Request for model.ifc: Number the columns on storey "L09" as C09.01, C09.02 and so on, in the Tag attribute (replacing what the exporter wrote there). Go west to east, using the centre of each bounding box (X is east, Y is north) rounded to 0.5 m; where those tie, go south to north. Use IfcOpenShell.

First a look at what the model holds.

```python
import ifcopenshell
import ifcopenshell.util.element
import ifcopenshell.util.placement

model = ifcopenshell.open("model.ifc")
print(model.schema)
storey = next(s for s in model.by_type("IfcBuildingStorey") if s.Name == "L09")
columns = [e for e in ifcopenshell.util.element.get_decomposition(storey) if e.is_a("IfcColumn")]
for e in sorted(columns, key=lambda e: e.id()):
    origin = ifcopenshell.util.placement.get_local_placement(e.ObjectPlacement)[:3, 3]
    print(e.id(), e.Tag, e.Name, origin.round(2) + 0.0, sep=" | ")
```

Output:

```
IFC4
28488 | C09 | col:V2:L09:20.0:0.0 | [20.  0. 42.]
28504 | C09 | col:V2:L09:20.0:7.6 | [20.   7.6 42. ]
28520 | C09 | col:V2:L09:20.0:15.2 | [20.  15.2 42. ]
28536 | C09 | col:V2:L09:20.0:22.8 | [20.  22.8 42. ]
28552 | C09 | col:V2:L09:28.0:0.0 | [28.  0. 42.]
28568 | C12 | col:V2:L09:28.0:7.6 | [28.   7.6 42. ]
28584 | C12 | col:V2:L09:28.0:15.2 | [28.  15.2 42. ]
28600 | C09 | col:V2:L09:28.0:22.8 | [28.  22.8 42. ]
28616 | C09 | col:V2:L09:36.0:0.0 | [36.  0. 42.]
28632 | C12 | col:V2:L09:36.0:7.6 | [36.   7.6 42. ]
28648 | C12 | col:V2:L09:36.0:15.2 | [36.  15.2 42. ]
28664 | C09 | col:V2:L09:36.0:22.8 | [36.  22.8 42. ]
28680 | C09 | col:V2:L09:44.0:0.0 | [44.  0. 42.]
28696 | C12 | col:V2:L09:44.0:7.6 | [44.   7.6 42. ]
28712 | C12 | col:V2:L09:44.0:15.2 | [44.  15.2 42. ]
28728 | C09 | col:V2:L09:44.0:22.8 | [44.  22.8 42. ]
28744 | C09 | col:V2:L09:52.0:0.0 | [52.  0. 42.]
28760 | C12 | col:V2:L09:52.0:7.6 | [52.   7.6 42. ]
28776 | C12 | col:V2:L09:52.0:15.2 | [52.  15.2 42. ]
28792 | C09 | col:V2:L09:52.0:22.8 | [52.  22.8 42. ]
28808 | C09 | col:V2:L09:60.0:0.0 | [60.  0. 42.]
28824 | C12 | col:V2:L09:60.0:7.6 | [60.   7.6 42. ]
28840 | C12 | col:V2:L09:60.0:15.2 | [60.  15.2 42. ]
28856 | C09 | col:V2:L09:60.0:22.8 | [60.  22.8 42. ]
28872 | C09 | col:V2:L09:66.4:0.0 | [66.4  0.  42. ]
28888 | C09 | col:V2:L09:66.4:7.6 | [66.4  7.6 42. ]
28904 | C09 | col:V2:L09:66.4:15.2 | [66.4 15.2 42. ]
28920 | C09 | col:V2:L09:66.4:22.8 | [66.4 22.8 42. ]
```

```python
import ifcopenshell
import ifcopenshell.geom
import ifcopenshell.util.element
import ifcopenshell.util.shape

model = ifcopenshell.open("model.ifc")
settings = ifcopenshell.geom.settings()
settings.set("use-world-coords", True)


def centre(element):
    shape = ifcopenshell.geom.create_shape(settings, element)
    return ifcopenshell.util.shape.get_bbox_centroid(shape.geometry)


storey = next(s for s in model.by_type("IfcBuildingStorey") if s.Name == "L09")
columns = [e for e in ifcopenshell.util.element.get_decomposition(storey) if e.is_a("IfcColumn")]

# Insertion points can sit at a corner or the storey origin, so sort by the geometry (in metres).
centres = {e: centre(e) for e in columns}
columns.sort(key=lambda e: (round(centres[e][0] / 0.5), centres[e][1]))

for i, e in enumerate(columns, start=1):
    number = f"C09.{i:02d}"
    e.Tag = number
    print(e.id(), number)

model.write("model_v2.ifc")
```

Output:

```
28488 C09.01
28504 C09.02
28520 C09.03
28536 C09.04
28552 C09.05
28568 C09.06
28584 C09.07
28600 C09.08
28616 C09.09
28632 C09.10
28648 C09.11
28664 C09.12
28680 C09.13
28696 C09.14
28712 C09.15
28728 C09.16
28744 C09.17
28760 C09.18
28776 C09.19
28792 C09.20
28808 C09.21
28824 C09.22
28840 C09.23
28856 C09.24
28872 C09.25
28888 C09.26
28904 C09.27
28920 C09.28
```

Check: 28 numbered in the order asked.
